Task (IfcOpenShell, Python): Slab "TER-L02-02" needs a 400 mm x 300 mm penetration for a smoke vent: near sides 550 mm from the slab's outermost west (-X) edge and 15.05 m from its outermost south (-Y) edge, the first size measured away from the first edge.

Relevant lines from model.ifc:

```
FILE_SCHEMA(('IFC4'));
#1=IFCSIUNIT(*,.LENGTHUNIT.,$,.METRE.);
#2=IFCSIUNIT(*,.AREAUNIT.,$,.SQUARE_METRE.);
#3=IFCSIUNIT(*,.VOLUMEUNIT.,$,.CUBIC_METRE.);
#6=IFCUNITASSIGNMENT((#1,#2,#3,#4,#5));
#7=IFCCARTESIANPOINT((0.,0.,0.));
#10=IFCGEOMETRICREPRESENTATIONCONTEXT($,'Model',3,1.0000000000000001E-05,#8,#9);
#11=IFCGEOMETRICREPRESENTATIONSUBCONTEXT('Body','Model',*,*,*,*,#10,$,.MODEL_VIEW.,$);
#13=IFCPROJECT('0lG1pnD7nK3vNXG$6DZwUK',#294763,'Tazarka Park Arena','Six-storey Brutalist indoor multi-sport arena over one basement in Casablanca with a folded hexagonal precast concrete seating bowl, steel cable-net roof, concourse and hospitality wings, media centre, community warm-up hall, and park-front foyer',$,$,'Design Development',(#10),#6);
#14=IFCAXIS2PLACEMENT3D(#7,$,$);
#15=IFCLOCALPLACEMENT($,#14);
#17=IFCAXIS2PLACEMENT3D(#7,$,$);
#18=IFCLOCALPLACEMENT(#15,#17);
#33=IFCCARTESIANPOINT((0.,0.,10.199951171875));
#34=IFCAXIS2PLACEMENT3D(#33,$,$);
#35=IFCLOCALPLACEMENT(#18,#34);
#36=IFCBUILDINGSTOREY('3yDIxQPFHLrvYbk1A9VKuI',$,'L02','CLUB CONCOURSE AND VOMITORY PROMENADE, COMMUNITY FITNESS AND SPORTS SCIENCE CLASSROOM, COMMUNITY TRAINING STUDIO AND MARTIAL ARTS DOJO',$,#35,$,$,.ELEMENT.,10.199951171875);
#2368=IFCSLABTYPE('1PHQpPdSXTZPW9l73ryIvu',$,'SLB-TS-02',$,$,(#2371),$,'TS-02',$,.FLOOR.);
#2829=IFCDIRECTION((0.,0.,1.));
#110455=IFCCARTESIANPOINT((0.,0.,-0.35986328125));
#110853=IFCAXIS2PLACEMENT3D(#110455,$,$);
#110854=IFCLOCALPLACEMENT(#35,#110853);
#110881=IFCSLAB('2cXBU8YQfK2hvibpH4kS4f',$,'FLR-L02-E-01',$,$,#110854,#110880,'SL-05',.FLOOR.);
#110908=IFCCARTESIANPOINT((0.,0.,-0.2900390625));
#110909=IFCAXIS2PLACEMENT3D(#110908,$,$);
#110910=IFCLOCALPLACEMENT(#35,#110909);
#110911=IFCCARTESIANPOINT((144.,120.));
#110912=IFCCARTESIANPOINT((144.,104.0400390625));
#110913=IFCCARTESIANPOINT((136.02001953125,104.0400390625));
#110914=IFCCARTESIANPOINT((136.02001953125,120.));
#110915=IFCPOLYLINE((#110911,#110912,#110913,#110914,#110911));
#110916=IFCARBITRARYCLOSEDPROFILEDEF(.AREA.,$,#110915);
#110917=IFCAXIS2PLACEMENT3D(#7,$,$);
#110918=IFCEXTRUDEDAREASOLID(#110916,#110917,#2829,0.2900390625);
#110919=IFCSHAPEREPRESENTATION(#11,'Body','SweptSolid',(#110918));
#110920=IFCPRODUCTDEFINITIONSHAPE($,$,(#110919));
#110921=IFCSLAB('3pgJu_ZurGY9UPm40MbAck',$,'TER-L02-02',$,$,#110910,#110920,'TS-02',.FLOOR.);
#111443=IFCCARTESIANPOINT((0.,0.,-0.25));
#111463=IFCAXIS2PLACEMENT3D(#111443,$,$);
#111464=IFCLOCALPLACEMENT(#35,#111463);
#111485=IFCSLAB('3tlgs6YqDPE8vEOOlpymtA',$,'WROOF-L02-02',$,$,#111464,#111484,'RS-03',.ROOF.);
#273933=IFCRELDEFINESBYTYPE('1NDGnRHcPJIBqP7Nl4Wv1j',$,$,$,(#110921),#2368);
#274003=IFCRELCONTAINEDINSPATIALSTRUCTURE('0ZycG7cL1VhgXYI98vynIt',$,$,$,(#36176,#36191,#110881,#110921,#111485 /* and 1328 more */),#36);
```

```python
import numpy as np
import ifcopenshell
import ifcopenshell.api.feature
import ifcopenshell.api.geometry
import ifcopenshell.api.root
import ifcopenshell.geom
import ifcopenshell.util.placement
import ifcopenshell.util.representation
import ifcopenshell.util.shape
import ifcopenshell.util.unit

model = ifcopenshell.open("model.ifc")
unit_scale = ifcopenshell.util.unit.calculate_unit_scale(model)
settings = ifcopenshell.geom.settings()


def volume(element):
    """Net volume in cubic metres, openings subtracted."""
    shape = ifcopenshell.geom.create_shape(settings, element)
    return ifcopenshell.util.shape.get_volume(shape.geometry)


slab = model.by_id(110921)
before = volume(slab)

# Extent in the slab's own axes, in metres. The edges named are its -X and -Y sides.
slab_shape = ifcopenshell.geom.create_shape(settings, slab)
vertices = ifcopenshell.util.shape.get_vertices(slab_shape.geometry)
x_min, y_min, bottom = vertices.min(axis=0)
top = vertices[:, 2].max()

opening = ifcopenshell.api.root.create_entity(model, ifc_class="IfcOpeningElement", name="Smoke vent opening", predefined_type="OPENING")
context = ifcopenshell.util.representation.get_context(model, "Model", "Body", "MODEL_VIEW")
width, depth = 0.4, 0.3
outline = [(0.0, 0.0), (width, 0.0), (width, depth), (0.0, depth), (0.0, 0.0)]
# Overshoot both faces by 50 mm so the cut is clean.
shape = ifcopenshell.api.geometry.add_slab_representation(
    model, context=context, depth=top - bottom + 0.1, polyline=outline
)
ifcopenshell.api.geometry.assign_representation(model, product=opening, representation=shape)

matrix = ifcopenshell.util.placement.get_local_placement(slab.ObjectPlacement)
matrix[:, 3] = matrix @ np.append(np.array([x_min + 0.55, y_min + 15.05, bottom - 0.05]) / unit_scale, 1.0)
ifcopenshell.api.geometry.edit_object_placement(model, product=opening, matrix=matrix, is_si=False)
ifcopenshell.api.feature.add_feature(model, feature=opening, element=slab)

after = volume(slab)

print(f"slab volume {before:.3f} -> {after:.3f} m3")

model.write("model_v2.ifc")
```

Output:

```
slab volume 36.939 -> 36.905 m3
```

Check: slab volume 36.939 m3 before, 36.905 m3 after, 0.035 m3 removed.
